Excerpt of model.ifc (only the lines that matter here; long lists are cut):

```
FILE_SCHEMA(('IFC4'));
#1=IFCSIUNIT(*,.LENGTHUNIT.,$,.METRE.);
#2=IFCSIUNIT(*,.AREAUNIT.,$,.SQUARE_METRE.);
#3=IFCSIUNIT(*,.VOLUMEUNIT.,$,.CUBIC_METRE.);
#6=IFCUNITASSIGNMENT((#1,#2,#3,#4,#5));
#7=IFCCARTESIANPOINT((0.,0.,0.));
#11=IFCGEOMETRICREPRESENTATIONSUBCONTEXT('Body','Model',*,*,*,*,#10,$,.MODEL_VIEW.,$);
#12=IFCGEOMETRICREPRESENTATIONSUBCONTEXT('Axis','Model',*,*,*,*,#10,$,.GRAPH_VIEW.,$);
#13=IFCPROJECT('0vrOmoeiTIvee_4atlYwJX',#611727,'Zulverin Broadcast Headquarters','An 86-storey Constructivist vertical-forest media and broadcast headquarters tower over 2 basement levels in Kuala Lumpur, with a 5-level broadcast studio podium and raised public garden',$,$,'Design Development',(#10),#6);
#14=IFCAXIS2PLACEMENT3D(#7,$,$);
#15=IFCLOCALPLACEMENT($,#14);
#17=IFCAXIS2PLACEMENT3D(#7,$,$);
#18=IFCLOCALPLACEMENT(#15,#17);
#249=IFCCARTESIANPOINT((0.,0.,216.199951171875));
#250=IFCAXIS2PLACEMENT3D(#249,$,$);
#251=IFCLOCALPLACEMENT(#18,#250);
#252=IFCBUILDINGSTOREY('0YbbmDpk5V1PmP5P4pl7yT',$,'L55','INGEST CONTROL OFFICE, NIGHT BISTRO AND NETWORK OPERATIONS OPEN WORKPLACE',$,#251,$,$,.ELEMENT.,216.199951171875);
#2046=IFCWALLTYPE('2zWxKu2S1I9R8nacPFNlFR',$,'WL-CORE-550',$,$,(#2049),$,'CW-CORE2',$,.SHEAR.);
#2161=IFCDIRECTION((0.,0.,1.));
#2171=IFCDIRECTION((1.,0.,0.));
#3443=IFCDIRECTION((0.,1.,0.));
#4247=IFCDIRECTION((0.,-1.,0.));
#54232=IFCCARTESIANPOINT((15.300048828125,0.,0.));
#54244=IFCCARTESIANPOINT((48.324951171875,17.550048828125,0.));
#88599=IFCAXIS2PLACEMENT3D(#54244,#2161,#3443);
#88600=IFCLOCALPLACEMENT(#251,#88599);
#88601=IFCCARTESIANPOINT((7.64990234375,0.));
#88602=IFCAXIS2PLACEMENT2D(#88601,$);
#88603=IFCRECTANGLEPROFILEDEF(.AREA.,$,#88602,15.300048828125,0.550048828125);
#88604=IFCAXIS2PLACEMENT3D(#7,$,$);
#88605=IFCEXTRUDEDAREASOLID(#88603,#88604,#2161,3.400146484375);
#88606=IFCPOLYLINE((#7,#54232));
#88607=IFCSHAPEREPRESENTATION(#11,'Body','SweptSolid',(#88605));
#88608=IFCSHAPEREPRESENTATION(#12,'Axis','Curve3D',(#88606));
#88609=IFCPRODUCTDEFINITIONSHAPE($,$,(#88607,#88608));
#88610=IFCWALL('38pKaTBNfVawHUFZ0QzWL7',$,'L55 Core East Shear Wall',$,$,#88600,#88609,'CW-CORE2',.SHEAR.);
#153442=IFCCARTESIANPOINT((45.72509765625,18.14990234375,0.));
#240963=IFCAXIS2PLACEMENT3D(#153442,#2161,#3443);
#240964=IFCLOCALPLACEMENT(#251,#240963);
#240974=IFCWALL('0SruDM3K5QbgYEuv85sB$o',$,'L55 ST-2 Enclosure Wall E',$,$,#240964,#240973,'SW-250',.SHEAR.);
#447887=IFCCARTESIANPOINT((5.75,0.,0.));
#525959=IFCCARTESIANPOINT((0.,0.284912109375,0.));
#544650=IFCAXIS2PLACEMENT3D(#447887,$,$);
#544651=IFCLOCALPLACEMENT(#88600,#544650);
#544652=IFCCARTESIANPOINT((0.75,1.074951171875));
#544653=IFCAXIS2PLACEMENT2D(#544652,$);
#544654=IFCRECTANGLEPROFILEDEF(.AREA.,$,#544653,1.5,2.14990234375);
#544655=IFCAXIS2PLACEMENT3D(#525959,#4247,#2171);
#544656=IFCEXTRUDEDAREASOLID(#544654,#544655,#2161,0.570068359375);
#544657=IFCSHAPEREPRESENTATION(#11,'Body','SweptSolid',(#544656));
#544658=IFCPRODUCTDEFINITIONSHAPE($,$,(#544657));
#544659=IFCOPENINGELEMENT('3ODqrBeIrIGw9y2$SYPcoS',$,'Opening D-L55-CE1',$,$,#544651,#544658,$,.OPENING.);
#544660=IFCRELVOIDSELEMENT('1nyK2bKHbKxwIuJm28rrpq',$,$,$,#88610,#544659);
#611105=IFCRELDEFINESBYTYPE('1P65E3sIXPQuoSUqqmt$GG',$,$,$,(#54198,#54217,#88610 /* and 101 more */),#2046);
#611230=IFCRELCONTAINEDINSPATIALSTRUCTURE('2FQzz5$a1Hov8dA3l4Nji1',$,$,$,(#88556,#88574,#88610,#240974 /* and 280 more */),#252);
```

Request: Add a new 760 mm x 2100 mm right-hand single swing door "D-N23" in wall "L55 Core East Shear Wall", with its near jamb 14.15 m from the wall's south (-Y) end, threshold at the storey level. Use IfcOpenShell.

```python
import numpy as np
import ifcopenshell
import ifcopenshell.api.feature
import ifcopenshell.api.geometry
import ifcopenshell.api.root
import ifcopenshell.api.spatial
import ifcopenshell.geom
import ifcopenshell.util.element
import ifcopenshell.util.placement
import ifcopenshell.util.representation
import ifcopenshell.util.shape
import ifcopenshell.util.unit

model = ifcopenshell.open("model.ifc")
unit_scale = ifcopenshell.util.unit.calculate_unit_scale(model)
settings = ifcopenshell.geom.settings()


def volume(element):
    """Net volume in cubic metres, openings subtracted."""
    shape = ifcopenshell.geom.create_shape(settings, element)
    return ifcopenshell.util.shape.get_volume(shape.geometry)


wall = model.by_guid("38pKaTBNfVawHUFZ0QzWL7")
storey = ifcopenshell.util.element.get_container(wall, ifc_class="IfcBuildingStorey")
context = ifcopenshell.util.representation.get_context(model, "Model", "Body", "MODEL_VIEW")
before = volume(wall)

width, height, from_end, sill = 0.76, 2.1, 14.15, 0.0  # metres

# The wall runs along its own X axis, and the end named is its -X end.
wall_shape = ifcopenshell.geom.create_shape(settings, wall)
x, y, z = ifcopenshell.util.shape.get_vertices(wall_shape.geometry).T
start = x.min() + from_end
face, thickness = float(y.min()), float(y.max() - y.min())
wall_matrix = ifcopenshell.util.placement.get_local_placement(wall.ObjectPlacement)
level = ifcopenshell.util.placement.get_local_placement(storey.ObjectPlacement)[2, 3]


def in_wall(x, y):
    """Placement at x, y metres in the wall's axes, at sill height."""
    matrix = wall_matrix.copy()
    matrix[:, 3] = wall_matrix @ np.array([x / unit_scale, y / unit_scale, 0.0, 1.0])
    matrix[2, 3] = level + sill / unit_scale
    return matrix


# Opening: a box that overshoots both wall faces by 50 mm.
opening = ifcopenshell.api.root.create_entity(model, ifc_class="IfcOpeningElement", predefined_type="OPENING")
box = ifcopenshell.api.geometry.add_wall_representation(
    model, context=context, length=width, height=height, thickness=thickness + 0.1
)
ifcopenshell.api.geometry.assign_representation(model, product=opening, representation=box)
ifcopenshell.api.geometry.edit_object_placement(model, product=opening, matrix=in_wall(start, face - 0.05), is_si=False)
ifcopenshell.api.feature.add_feature(model, feature=opening, element=wall)

door = ifcopenshell.api.root.create_entity(model, ifc_class="IfcDoor", name="D-N23", predefined_type="DOOR")
door.OverallWidth, door.OverallHeight = width / unit_scale, height / unit_scale
door.OperationType = "SINGLE_SWING_RIGHT"
body = ifcopenshell.api.geometry.add_door_representation(
    model,
    context=context,
    overall_width=door.OverallWidth,
    overall_height=door.OverallHeight,
    operation_type="SINGLE_SWING_RIGHT",
    lining_properties={"LiningDepth": thickness / unit_scale, "ThresholdDepth": thickness / unit_scale},
)
ifcopenshell.api.geometry.assign_representation(model, product=door, representation=body)
ifcopenshell.api.spatial.assign_container(model, products=[door], relating_structure=storey)
ifcopenshell.api.feature.add_filling(model, opening=opening, element=door)

# The lining spans the wall, so the door starts at the wall face.
ifcopenshell.api.geometry.edit_object_placement(model, product=door, matrix=in_wall(start, face), is_si=False)

after = volume(wall)

print(f"wall volume {before:.3f} -> {after:.3f} m3")

model.write("model_edited.ifc")
```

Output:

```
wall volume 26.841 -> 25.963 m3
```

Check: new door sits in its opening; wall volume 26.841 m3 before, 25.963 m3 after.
